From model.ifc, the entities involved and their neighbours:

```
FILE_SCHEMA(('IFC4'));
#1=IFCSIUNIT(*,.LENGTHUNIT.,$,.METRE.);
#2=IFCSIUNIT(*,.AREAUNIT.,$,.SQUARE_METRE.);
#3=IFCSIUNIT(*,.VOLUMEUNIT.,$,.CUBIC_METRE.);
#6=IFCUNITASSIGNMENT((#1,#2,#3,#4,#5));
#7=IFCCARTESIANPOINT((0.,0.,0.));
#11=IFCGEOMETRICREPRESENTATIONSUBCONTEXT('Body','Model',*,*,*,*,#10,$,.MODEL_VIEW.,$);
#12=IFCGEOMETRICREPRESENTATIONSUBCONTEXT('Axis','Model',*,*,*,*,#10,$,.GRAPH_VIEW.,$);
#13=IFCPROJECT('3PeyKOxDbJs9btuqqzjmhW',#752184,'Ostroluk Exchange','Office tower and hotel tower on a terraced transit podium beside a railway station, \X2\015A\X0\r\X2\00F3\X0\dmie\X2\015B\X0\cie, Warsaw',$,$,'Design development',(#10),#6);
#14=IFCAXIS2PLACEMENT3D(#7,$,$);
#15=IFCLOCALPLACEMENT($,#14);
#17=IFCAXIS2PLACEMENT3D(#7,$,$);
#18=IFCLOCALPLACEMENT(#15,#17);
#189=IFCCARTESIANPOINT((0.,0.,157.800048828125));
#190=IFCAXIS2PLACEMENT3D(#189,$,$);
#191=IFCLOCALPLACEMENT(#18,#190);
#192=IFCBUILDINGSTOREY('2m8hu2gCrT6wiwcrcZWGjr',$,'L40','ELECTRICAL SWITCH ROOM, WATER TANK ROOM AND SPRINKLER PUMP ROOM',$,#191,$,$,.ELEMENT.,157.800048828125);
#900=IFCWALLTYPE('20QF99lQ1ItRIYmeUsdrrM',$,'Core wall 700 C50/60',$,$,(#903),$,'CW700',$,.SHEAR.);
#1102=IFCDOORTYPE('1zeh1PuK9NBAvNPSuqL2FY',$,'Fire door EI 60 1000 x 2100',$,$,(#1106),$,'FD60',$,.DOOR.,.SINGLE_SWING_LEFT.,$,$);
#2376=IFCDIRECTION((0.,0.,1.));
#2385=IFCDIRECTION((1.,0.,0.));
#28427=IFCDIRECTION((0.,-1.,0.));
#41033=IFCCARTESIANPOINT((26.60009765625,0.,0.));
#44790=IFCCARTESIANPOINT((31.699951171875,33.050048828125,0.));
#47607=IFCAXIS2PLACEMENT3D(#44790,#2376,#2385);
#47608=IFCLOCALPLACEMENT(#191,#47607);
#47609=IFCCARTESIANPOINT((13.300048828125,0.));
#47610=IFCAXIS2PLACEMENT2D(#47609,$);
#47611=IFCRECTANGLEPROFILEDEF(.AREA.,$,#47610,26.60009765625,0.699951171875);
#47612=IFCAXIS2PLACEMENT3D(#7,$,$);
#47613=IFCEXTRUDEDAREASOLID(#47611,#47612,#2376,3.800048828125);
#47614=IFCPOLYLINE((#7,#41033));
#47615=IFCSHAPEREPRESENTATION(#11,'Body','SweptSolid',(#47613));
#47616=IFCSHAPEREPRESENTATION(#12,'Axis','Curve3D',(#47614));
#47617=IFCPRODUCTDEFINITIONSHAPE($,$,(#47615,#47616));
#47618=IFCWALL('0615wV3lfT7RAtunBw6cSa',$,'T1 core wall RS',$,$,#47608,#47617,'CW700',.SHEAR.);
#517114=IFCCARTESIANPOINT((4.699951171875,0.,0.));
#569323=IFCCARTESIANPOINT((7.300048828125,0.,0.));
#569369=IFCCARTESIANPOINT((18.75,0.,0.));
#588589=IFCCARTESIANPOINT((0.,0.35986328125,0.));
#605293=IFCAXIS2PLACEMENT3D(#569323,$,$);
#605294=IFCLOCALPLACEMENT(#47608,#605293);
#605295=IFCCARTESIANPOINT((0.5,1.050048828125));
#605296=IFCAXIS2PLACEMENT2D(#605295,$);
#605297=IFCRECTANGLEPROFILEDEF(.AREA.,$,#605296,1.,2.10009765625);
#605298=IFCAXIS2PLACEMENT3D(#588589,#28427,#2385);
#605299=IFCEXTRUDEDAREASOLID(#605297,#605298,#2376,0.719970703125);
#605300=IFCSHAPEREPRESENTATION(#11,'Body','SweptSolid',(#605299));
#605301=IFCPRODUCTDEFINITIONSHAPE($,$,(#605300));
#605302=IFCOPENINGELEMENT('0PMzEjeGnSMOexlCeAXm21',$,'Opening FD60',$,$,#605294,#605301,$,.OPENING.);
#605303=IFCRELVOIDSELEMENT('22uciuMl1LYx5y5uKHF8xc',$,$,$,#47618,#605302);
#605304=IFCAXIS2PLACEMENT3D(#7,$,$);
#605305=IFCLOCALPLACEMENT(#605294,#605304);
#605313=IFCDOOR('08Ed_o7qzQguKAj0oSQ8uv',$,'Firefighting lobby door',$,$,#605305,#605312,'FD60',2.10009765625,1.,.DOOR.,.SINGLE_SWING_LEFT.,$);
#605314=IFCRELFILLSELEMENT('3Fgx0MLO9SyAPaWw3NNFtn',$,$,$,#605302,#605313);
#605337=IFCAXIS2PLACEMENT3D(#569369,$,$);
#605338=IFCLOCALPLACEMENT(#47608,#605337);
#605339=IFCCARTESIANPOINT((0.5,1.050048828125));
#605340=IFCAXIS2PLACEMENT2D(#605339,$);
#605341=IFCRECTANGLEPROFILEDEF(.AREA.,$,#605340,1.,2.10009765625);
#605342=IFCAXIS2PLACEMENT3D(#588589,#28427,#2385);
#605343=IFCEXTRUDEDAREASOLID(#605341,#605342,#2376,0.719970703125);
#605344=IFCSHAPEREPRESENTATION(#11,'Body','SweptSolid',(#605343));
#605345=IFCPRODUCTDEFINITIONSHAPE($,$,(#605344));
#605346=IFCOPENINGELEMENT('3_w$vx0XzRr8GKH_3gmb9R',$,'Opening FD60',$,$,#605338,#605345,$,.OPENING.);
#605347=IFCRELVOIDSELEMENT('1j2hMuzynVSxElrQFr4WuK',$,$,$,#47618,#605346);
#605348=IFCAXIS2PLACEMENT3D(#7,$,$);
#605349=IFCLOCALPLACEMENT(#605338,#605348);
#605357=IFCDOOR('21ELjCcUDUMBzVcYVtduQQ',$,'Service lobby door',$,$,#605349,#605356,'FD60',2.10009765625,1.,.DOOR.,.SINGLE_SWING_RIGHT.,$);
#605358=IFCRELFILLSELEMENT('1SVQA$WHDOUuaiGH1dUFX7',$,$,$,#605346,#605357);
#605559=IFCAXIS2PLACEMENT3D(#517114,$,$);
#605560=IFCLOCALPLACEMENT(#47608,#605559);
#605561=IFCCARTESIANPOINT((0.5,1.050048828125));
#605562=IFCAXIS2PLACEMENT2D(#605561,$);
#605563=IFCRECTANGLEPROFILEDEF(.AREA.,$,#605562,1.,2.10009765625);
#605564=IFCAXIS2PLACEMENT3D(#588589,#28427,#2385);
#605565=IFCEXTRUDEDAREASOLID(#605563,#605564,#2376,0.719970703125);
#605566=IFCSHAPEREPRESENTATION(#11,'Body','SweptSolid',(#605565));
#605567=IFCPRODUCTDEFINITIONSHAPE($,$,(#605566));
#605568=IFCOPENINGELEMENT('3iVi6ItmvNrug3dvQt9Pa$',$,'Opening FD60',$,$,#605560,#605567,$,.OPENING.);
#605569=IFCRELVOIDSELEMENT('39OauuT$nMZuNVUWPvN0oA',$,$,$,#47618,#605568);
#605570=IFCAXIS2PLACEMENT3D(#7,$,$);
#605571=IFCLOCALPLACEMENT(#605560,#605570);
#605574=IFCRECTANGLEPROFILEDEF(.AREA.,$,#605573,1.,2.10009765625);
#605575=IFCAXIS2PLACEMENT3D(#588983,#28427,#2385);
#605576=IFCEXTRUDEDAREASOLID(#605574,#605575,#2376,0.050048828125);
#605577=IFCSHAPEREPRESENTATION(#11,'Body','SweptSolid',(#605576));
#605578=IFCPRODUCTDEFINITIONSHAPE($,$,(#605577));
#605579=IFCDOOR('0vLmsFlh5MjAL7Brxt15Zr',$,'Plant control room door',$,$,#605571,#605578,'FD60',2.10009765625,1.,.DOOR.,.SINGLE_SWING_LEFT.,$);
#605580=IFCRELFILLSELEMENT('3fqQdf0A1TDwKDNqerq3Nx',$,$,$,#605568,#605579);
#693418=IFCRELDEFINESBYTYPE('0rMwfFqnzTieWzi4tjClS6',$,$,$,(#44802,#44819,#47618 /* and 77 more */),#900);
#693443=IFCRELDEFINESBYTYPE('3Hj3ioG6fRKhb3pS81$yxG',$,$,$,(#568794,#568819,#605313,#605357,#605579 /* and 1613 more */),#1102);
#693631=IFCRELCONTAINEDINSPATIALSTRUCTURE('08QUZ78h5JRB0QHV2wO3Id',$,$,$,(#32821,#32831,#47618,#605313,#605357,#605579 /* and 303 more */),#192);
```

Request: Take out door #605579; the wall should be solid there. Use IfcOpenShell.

```python
import ifcopenshell
import ifcopenshell.api.feature
import ifcopenshell.api.root
import ifcopenshell.geom
import ifcopenshell.util.shape

model = ifcopenshell.open("model.ifc")
settings = ifcopenshell.geom.settings()


def volume(element):
    """Net volume in cubic metres, openings subtracted."""
    shape = ifcopenshell.geom.create_shape(settings, element)
    return ifcopenshell.util.shape.get_volume(shape.geometry)


door = model.by_guid("0vLmsFlh5MjAL7Brxt15Zr")
opening = door.FillsVoids[0].RelatingOpeningElement
wall = opening.VoidsElements[0].RelatingBuildingElement
before = volume(wall)

ifcopenshell.api.root.remove_product(model, product=door)
ifcopenshell.api.feature.remove_feature(model, feature=opening)

after = volume(wall)

print(f"wall volume {before:.3f} -> {after:.3f} m3")

model.write("model-out.ifc")
```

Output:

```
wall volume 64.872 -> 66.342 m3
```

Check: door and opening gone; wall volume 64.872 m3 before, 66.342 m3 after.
